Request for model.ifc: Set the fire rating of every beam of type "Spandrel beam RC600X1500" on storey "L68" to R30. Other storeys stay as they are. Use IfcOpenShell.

First a look at what the model holds.

```python
import ifcopenshell
import ifcopenshell.util.element

model = ifcopenshell.open("model.ifc")
print(model.schema)
storey = next(s for s in model.by_type("IfcBuildingStorey") if s.Name == "L68")
beams = [e for e in ifcopenshell.util.element.get_decomposition(storey) if e.is_a("IfcBeam")]
seen = {}
for e in beams:
    element_type = ifcopenshell.util.element.get_type(e)
    key = (element_type.Name if element_type != e and element_type else None, ifcopenshell.util.element.get_pset(e, "Pset_BeamCommon", "FireRating"))
    seen[key] = seen.get(key, 0) + 1
for (name, value), count in sorted(seen.items(), key=str):
    print(count, "x", name, "|", value)
```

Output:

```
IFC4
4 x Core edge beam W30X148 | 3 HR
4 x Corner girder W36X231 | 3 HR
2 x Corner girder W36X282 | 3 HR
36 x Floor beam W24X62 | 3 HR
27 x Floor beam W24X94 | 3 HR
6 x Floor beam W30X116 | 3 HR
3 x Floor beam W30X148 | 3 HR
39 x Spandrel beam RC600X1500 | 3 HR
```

```python
import ifcopenshell
import ifcopenshell.api.pset
import ifcopenshell.util.element

model = ifcopenshell.open("model.ifc")

storey = next(s for s in model.by_type("IfcBuildingStorey") if s.Name == "L68")
beams = [e for e in ifcopenshell.util.element.get_decomposition(storey) if e.is_a("IfcBeam")]

count = 0
for e in beams:
    element_type = ifcopenshell.util.element.get_type(e)
    if element_type in (None, e) or element_type.Name != "Spandrel beam RC600X1500":
        continue
    found = ifcopenshell.util.element.get_pset(e, "Pset_BeamCommon", should_inherit=False)
    if found:
        pset = model.by_id(found["id"])
        if len(ifcopenshell.util.element.get_elements_by_pset(pset)) > 1:
            pset = ifcopenshell.api.pset.unshare_pset(model, products=[e], pset=pset)[0]
    else:
        pset = ifcopenshell.api.pset.add_pset(model, product=e, name="Pset_BeamCommon")
    ifcopenshell.api.pset.edit_pset(model, pset=pset, properties={"FireRating": "R30"})
    count += 1

print(count, "beams updated")

model.write("model_edited.ifc")
```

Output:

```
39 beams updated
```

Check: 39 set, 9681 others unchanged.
